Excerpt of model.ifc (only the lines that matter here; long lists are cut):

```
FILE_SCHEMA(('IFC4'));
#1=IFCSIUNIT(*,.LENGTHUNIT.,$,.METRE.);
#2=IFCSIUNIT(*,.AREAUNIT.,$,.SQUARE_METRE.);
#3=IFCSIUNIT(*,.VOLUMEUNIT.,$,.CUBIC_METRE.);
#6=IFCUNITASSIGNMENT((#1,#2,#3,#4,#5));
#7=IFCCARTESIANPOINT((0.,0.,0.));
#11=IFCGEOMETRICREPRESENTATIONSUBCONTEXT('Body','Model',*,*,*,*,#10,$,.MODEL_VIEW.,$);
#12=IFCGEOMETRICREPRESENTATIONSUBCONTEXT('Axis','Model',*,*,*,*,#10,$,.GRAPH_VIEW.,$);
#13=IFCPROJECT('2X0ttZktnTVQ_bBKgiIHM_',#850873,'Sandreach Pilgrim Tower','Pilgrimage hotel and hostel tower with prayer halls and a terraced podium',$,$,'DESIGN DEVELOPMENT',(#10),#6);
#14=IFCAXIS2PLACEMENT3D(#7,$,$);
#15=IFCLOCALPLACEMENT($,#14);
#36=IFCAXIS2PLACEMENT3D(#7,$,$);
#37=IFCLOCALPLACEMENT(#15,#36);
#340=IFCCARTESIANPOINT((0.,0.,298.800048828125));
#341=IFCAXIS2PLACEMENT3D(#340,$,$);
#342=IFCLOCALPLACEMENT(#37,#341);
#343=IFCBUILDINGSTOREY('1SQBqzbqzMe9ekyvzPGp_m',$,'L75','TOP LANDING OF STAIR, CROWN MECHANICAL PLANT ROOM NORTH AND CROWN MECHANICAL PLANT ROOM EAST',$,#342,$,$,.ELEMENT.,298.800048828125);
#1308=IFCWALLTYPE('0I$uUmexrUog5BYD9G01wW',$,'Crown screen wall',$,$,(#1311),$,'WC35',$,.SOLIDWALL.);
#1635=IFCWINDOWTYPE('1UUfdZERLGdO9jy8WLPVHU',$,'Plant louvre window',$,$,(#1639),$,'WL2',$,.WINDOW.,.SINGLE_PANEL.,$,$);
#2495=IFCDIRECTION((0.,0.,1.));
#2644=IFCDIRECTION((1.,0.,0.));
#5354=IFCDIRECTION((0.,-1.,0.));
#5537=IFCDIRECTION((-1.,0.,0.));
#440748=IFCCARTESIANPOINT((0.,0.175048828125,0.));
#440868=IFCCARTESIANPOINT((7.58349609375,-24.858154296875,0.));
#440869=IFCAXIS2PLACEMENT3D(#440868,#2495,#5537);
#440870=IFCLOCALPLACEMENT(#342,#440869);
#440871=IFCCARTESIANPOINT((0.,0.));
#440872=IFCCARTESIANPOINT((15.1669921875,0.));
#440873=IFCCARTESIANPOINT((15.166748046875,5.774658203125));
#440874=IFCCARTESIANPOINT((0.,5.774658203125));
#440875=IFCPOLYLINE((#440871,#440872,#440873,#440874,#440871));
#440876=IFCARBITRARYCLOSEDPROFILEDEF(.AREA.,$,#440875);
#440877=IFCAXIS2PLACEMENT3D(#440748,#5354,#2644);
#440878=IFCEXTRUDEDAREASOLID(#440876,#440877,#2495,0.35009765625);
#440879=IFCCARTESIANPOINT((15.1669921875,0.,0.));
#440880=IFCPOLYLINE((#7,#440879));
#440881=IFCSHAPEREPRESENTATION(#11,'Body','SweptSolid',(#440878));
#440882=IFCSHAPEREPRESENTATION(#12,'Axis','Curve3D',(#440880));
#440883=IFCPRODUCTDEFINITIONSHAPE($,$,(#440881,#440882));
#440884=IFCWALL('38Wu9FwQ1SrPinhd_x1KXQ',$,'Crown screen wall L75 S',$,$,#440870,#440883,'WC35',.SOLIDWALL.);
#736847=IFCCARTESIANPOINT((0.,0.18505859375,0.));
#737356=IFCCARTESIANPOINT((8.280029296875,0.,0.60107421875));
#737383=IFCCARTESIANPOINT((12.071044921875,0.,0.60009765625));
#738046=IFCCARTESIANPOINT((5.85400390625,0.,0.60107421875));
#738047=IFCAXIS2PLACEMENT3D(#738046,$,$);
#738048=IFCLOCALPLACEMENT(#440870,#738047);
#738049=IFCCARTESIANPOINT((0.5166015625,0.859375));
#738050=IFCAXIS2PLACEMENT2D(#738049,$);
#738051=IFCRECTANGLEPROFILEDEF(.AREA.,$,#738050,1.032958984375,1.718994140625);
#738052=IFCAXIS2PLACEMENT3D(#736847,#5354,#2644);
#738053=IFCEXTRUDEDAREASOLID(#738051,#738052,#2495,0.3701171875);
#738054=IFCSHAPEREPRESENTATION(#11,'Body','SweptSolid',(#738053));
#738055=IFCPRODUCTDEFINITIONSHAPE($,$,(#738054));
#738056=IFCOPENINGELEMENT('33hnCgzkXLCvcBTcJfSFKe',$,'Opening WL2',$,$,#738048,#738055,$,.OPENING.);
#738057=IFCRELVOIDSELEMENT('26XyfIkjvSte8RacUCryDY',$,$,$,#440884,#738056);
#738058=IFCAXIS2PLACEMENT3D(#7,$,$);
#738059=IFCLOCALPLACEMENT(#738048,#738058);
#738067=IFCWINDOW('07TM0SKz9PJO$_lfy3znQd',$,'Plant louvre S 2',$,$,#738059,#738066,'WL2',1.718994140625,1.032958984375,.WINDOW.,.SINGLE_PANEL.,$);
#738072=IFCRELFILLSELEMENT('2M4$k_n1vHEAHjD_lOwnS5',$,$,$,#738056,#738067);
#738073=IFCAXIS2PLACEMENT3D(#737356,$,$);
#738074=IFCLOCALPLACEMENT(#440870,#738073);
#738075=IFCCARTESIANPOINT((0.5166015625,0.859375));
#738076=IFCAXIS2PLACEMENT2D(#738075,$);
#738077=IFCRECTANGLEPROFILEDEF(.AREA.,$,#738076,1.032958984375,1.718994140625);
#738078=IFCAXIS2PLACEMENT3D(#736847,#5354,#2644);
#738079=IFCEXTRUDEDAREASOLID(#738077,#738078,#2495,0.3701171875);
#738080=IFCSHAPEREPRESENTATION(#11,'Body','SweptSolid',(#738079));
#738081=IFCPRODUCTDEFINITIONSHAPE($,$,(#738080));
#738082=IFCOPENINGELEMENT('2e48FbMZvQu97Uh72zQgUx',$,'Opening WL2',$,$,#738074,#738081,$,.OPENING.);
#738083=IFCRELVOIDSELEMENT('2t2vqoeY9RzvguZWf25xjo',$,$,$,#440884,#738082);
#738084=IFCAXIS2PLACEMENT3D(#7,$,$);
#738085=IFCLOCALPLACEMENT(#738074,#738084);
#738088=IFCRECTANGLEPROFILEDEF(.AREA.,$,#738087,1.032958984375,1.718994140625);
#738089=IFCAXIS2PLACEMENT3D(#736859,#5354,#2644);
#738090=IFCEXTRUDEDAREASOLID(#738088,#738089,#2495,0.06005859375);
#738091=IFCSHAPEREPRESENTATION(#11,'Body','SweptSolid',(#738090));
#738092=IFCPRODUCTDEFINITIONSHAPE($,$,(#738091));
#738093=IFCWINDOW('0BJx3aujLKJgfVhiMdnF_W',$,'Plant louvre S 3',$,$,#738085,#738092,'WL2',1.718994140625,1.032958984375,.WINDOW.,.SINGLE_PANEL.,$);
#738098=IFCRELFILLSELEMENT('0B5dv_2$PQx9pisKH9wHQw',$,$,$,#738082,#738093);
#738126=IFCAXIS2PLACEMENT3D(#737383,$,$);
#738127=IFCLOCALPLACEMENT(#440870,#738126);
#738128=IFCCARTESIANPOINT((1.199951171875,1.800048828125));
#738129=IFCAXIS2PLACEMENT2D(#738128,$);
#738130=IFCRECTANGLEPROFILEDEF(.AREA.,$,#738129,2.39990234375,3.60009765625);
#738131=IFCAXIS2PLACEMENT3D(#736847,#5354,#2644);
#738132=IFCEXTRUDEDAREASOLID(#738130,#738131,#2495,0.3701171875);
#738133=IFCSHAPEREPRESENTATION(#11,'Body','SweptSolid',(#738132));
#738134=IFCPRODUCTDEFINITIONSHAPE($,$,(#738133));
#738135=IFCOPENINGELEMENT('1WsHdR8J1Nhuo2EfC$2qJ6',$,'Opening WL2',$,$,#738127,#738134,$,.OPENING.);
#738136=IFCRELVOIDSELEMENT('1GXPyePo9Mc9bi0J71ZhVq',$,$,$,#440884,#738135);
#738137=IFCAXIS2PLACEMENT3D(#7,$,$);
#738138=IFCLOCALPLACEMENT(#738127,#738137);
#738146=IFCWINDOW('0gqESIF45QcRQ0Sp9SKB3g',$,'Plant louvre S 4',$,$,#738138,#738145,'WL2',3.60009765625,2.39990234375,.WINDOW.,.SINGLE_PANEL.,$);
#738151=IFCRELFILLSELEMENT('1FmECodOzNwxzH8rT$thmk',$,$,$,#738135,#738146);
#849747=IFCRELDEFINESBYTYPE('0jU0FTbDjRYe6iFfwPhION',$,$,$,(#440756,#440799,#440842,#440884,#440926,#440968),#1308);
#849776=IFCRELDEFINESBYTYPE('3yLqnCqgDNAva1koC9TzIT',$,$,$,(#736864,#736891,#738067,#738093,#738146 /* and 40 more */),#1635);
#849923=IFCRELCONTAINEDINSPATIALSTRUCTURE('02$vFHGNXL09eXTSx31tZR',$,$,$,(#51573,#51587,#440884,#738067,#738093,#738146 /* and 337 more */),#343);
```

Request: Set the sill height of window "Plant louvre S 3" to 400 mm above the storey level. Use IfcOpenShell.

```python
import numpy as np
import ifcopenshell
import ifcopenshell.api.geometry
import ifcopenshell.geom
import ifcopenshell.util.element
import ifcopenshell.util.placement
import ifcopenshell.util.shape
import ifcopenshell.util.unit

model = ifcopenshell.open("model.ifc")
unit_scale = ifcopenshell.util.unit.calculate_unit_scale(model)

window = model.by_guid("0BJx3aujLKJgfVhiMdnF_W")
opening = window.FillsVoids[0].RelatingOpeningElement
storey = ifcopenshell.util.element.get_container(window, ifc_class="IfcBuildingStorey")
level = ifcopenshell.util.placement.get_local_placement(storey.ObjectPlacement)[2, 3]

# The opening's origin need not be at the sill, so measure its lowest point.
shape = ifcopenshell.geom.create_shape(ifcopenshell.geom.settings(), opening)
bottom = ifcopenshell.util.shape.get_shape_bottom_elevation(shape, shape.geometry) / unit_scale
dz = level + 0.4 / unit_scale - bottom

shift = np.array([0.0, 0.0, dz])
# The window is placed relative to its opening, so it follows when the opening moves.
matrix = ifcopenshell.util.placement.get_local_placement(opening.ObjectPlacement)
matrix[:3, 3] += shift
ifcopenshell.api.geometry.edit_object_placement(
    model, product=opening, matrix=matrix, is_si=False, should_transform_children=True
)

print(f"moved by {dz * unit_scale:+.3f} m")

model.write("model-out.ifc")
```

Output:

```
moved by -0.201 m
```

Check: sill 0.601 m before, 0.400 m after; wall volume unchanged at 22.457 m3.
